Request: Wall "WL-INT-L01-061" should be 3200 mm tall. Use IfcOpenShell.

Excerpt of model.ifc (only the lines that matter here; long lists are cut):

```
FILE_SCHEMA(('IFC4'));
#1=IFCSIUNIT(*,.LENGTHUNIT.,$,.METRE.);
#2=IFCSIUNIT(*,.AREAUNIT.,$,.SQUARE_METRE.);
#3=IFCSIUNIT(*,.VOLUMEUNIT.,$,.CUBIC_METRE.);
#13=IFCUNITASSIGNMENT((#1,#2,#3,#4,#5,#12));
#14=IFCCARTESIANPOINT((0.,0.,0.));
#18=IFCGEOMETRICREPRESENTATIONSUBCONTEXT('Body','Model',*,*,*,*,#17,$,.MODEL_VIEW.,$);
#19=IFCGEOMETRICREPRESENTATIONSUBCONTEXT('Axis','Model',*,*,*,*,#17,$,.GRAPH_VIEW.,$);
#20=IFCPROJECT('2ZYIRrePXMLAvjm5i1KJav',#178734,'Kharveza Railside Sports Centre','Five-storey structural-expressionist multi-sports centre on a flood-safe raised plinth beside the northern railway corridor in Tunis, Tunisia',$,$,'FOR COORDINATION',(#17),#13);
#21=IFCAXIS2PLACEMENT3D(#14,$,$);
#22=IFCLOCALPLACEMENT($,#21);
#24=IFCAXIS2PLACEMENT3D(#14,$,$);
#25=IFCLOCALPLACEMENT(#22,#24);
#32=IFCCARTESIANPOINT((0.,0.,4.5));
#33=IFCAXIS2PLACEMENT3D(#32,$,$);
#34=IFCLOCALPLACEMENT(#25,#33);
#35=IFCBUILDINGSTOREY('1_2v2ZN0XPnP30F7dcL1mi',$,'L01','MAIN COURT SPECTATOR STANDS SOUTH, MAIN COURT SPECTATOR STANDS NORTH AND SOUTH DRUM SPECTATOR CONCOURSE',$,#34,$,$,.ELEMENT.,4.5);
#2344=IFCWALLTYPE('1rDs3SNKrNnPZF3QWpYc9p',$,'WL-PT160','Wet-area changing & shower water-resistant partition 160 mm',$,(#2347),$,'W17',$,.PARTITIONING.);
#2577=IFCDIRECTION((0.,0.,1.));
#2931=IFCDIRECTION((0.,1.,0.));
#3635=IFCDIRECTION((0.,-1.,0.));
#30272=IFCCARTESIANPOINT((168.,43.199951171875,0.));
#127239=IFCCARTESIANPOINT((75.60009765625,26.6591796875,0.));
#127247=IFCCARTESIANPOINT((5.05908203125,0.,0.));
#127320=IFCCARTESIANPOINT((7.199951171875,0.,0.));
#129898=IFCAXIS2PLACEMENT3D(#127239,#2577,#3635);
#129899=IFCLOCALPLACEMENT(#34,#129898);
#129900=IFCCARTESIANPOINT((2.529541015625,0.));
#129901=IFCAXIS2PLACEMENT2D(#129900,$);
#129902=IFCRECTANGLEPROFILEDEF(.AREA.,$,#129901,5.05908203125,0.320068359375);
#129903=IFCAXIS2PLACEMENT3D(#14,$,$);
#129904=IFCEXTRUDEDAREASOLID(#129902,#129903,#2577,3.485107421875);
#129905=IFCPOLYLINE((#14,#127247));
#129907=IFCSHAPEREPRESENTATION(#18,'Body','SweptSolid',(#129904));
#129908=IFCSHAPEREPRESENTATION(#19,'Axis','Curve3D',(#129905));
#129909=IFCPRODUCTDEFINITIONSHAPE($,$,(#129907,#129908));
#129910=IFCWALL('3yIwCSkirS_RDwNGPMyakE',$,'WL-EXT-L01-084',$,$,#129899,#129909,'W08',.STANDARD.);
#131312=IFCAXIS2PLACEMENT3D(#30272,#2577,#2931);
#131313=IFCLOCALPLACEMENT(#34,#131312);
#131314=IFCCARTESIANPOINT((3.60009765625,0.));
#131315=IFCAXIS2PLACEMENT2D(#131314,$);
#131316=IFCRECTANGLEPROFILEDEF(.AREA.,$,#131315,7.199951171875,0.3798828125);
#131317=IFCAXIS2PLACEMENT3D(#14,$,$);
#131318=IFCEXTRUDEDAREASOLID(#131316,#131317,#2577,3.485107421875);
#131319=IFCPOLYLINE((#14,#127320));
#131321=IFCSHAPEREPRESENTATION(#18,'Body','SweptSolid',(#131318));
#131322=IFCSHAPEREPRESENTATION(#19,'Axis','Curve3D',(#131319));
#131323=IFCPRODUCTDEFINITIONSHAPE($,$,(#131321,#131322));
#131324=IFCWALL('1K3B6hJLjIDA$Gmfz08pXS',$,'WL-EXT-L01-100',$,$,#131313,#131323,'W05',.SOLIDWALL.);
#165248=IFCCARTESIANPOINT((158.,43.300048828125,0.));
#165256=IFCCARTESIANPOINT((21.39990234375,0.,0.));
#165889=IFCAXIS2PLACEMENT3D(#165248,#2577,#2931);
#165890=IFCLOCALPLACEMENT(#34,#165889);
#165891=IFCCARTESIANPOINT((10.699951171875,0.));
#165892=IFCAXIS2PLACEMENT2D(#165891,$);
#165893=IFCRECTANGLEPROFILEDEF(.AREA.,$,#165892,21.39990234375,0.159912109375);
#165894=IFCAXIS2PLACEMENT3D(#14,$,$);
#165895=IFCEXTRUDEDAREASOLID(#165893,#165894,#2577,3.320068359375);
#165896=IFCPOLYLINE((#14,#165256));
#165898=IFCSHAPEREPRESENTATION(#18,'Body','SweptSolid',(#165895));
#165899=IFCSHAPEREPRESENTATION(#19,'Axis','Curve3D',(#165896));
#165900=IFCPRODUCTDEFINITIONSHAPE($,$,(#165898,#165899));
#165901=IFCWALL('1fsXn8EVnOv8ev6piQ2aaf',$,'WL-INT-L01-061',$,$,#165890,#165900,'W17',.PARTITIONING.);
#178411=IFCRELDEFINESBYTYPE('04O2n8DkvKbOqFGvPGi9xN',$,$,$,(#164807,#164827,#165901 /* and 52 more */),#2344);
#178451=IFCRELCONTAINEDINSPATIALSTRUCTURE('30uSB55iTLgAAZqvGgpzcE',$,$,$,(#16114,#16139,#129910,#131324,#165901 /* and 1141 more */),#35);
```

```python
import ifcopenshell
import ifcopenshell.geom
import ifcopenshell.util.representation
import ifcopenshell.util.shape
import ifcopenshell.util.unit

model = ifcopenshell.open("model.ifc")
unit_scale = ifcopenshell.util.unit.calculate_unit_scale(model)
settings = ifcopenshell.geom.settings()


def volume(element):
    """Net volume in cubic metres, openings subtracted."""
    shape = ifcopenshell.geom.create_shape(settings, element)
    return ifcopenshell.util.shape.get_volume(shape.geometry)


wall = model.by_id(165901)
before = volume(wall)

body = ifcopenshell.util.representation.get_representation(wall, "Model", "Body")
solid = body.Items[0]
old_height = solid.Depth
solid.Depth = 3.2 / unit_scale
after = volume(wall)

print(f"height {old_height:g} -> {solid.Depth:g}, volume {before:.3f} -> {after:.3f} m3")

model.write("model_updated.ifc")
```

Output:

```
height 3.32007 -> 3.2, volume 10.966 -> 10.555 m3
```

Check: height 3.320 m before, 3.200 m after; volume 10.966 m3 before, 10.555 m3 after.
